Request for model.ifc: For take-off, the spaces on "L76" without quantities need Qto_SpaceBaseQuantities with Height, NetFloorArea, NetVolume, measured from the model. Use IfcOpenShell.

First a look at what the model holds.

```python
import ifcopenshell
import ifcopenshell.util.element
import ifcopenshell.util.unit

model = ifcopenshell.open("model.ifc")
print(model.schema)
for unit_type in ("LENGTHUNIT", "AREAUNIT", "VOLUMEUNIT"):
    print(unit_type, ifcopenshell.util.unit.calculate_unit_scale(model, unit_type))
storey = next(s for s in model.by_type("IfcBuildingStorey") if s.Name == "L76")
spaces = [e for e in ifcopenshell.util.element.get_decomposition(storey) if e.is_a("IfcSpace")]
for e in sorted(spaces, key=lambda e: e.id()):
    print(e.id(), e.is_a(), e.Name, list(ifcopenshell.util.element.get_psets(e, qtos_only=True)), sep=" | ")
```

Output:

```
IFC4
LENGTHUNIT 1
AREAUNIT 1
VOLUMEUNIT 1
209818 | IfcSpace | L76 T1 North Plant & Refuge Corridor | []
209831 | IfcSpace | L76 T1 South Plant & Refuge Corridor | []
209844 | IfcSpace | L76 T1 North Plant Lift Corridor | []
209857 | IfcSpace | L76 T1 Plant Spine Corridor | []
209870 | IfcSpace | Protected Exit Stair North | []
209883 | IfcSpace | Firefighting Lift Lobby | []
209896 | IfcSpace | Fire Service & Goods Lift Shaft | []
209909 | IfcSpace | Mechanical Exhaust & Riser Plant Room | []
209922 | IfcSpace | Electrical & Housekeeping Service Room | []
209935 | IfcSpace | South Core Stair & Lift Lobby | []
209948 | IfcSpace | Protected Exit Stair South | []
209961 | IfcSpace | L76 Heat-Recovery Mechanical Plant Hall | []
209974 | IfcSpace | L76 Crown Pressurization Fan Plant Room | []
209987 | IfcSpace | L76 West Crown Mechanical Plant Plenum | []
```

```python
import ifcopenshell
import ifcopenshell.api.pset
import ifcopenshell.geom
import ifcopenshell.util.element
import ifcopenshell.util.shape
import ifcopenshell.util.unit

model = ifcopenshell.open("model.ifc")
unit_scale = ifcopenshell.util.unit.calculate_unit_scale(model)
area_scale = ifcopenshell.util.unit.calculate_unit_scale(model, "AREAUNIT")
volume_scale = ifcopenshell.util.unit.calculate_unit_scale(model, "VOLUMEUNIT")
settings = ifcopenshell.geom.settings()

storey = next(s for s in model.by_type("IfcBuildingStorey") if s.Name == "L76")
spaces = [e for e in ifcopenshell.util.element.get_decomposition(storey) if e.is_a("IfcSpace")]

for e in sorted(spaces, key=lambda e: e.id()):
    if ifcopenshell.util.element.get_psets(e, qtos_only=True, should_inherit=False):
        continue
    # Geometry comes back in metres, in the element's own axes.
    shape = ifcopenshell.geom.create_shape(settings, e)
    values = {
        "Height": ifcopenshell.util.shape.get_z(shape.geometry) / unit_scale,
        "NetFloorArea": ifcopenshell.util.shape.get_footprint_area(shape.geometry) / area_scale,
        "NetVolume": ifcopenshell.util.shape.get_volume(shape.geometry) / volume_scale,
    }
    qto = ifcopenshell.api.pset.add_qto(model, product=e, name="Qto_SpaceBaseQuantities")
    ifcopenshell.api.pset.edit_qto(model, qto=qto, properties=values)
    print(e.id(), {k: round(v, 3) for k, v in values.items()})

model.write("model_v2.ifc")
```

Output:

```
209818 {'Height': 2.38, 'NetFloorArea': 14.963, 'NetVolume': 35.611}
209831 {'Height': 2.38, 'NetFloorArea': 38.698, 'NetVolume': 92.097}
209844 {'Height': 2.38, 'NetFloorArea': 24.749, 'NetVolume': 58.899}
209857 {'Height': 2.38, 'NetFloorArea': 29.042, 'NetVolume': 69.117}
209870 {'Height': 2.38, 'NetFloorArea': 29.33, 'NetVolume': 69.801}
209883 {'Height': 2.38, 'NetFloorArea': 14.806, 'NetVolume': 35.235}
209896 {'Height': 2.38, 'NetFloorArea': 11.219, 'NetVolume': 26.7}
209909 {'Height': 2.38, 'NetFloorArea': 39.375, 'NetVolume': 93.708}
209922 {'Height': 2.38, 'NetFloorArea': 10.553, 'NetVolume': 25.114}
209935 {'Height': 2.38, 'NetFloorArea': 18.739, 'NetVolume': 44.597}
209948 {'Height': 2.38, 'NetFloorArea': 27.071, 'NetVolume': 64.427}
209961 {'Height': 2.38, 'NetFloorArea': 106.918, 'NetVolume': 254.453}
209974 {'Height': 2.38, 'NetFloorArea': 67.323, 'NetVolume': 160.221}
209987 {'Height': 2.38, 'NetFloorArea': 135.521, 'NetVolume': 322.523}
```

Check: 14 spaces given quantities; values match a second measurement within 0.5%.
